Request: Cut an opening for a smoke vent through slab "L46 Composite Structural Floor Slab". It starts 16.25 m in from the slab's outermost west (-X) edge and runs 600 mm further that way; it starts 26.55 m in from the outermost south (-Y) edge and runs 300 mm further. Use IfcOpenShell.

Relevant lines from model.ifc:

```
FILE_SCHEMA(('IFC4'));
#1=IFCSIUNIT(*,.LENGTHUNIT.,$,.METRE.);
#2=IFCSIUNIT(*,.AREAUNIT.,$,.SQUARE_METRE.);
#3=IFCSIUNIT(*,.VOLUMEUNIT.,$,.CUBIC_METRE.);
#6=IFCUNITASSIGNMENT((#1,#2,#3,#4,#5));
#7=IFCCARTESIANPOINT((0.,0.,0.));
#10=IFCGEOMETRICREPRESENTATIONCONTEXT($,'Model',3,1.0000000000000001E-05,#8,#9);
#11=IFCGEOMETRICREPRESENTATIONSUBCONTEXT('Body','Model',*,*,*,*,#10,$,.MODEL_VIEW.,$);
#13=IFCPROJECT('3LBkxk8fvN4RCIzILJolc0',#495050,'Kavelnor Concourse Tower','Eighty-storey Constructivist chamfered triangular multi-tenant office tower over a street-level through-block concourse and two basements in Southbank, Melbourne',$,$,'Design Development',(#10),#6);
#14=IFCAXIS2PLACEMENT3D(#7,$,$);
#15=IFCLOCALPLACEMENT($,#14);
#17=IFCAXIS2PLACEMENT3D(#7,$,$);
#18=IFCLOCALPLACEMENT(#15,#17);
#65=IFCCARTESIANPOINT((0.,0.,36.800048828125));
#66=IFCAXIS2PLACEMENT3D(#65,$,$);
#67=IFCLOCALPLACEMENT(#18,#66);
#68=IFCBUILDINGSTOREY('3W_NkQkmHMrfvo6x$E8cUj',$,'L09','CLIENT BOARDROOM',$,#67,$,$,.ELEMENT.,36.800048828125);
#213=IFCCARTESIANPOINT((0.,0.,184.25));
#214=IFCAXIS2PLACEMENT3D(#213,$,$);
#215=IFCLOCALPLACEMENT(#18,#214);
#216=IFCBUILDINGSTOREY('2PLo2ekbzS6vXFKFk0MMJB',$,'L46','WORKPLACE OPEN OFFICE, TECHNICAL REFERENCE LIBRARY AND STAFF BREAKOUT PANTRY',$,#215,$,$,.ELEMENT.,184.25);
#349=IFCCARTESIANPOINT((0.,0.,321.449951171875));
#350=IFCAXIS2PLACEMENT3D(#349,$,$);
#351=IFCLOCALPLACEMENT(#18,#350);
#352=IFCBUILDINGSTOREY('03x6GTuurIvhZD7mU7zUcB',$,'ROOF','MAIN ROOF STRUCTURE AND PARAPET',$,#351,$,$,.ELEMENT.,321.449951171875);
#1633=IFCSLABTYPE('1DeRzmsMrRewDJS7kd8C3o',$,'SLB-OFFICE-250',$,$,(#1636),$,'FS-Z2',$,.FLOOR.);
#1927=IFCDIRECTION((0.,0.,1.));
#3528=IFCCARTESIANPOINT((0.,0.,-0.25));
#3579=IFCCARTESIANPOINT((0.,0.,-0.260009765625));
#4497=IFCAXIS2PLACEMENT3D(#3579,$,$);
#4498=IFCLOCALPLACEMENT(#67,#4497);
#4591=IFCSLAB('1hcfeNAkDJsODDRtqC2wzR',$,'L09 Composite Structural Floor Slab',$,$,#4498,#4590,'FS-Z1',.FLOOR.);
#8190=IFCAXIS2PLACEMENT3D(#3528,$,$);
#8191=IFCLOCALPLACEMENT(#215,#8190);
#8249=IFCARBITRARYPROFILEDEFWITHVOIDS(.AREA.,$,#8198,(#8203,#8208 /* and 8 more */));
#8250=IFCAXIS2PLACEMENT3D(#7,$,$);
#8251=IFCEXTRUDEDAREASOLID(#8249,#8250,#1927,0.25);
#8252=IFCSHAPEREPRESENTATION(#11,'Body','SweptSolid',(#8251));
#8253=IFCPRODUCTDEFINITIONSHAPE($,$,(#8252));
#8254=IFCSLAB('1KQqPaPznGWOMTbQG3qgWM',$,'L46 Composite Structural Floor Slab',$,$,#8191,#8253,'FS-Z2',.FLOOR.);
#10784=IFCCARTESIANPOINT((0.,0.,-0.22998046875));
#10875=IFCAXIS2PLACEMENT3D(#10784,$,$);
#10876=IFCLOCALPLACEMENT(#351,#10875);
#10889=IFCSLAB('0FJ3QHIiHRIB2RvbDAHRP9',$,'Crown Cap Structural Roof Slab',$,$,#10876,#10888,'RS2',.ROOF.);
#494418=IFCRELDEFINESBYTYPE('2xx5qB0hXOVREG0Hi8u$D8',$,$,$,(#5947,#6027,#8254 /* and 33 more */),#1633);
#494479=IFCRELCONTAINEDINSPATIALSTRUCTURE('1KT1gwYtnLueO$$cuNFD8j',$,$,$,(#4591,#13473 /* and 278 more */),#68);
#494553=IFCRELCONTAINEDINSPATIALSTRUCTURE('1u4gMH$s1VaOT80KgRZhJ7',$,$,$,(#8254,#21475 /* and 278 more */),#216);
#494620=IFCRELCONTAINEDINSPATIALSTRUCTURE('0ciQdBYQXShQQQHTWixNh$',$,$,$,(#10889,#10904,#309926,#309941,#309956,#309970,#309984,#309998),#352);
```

```python
import numpy as np
import ifcopenshell
import ifcopenshell.api.feature
import ifcopenshell.api.geometry
import ifcopenshell.api.root
import ifcopenshell.geom
import ifcopenshell.util.placement
import ifcopenshell.util.representation
import ifcopenshell.util.shape
import ifcopenshell.util.unit

model = ifcopenshell.open("model.ifc")
unit_scale = ifcopenshell.util.unit.calculate_unit_scale(model)
settings = ifcopenshell.geom.settings()


def volume(element):
    """Net volume in cubic metres, openings subtracted."""
    shape = ifcopenshell.geom.create_shape(settings, element)
    return ifcopenshell.util.shape.get_volume(shape.geometry)


slab = model.by_guid("1KQqPaPznGWOMTbQG3qgWM")
before = volume(slab)

# Extent in the slab's own axes, in metres. The edges named are its -X and -Y sides.
slab_shape = ifcopenshell.geom.create_shape(settings, slab)
vertices = ifcopenshell.util.shape.get_vertices(slab_shape.geometry)
x_min, y_min, bottom = vertices.min(axis=0)
top = vertices[:, 2].max()

opening = ifcopenshell.api.root.create_entity(model, ifc_class="IfcOpeningElement", name="Smoke vent opening", predefined_type="OPENING")
context = ifcopenshell.util.representation.get_context(model, "Model", "Body", "MODEL_VIEW")
width, depth = 0.6, 0.3
outline = [(0.0, 0.0), (width, 0.0), (width, depth), (0.0, depth), (0.0, 0.0)]
# Overshoot both faces by 50 mm so the cut is clean.
shape = ifcopenshell.api.geometry.add_slab_representation(
    model, context=context, depth=top - bottom + 0.1, polyline=outline
)
ifcopenshell.api.geometry.assign_representation(model, product=opening, representation=shape)

matrix = ifcopenshell.util.placement.get_local_placement(slab.ObjectPlacement)
matrix[:, 3] = matrix @ np.append(np.array([x_min + 16.25, y_min + 26.55, bottom - 0.05]) / unit_scale, 1.0)
ifcopenshell.api.geometry.edit_object_placement(model, product=opening, matrix=matrix, is_si=False)
ifcopenshell.api.feature.add_feature(model, feature=opening, element=slab)

after = volume(slab)

print(f"slab volume {before:.3f} -> {after:.3f} m3")

model.write("model_rev.ifc")
```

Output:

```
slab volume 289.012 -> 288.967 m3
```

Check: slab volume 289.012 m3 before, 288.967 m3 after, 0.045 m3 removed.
